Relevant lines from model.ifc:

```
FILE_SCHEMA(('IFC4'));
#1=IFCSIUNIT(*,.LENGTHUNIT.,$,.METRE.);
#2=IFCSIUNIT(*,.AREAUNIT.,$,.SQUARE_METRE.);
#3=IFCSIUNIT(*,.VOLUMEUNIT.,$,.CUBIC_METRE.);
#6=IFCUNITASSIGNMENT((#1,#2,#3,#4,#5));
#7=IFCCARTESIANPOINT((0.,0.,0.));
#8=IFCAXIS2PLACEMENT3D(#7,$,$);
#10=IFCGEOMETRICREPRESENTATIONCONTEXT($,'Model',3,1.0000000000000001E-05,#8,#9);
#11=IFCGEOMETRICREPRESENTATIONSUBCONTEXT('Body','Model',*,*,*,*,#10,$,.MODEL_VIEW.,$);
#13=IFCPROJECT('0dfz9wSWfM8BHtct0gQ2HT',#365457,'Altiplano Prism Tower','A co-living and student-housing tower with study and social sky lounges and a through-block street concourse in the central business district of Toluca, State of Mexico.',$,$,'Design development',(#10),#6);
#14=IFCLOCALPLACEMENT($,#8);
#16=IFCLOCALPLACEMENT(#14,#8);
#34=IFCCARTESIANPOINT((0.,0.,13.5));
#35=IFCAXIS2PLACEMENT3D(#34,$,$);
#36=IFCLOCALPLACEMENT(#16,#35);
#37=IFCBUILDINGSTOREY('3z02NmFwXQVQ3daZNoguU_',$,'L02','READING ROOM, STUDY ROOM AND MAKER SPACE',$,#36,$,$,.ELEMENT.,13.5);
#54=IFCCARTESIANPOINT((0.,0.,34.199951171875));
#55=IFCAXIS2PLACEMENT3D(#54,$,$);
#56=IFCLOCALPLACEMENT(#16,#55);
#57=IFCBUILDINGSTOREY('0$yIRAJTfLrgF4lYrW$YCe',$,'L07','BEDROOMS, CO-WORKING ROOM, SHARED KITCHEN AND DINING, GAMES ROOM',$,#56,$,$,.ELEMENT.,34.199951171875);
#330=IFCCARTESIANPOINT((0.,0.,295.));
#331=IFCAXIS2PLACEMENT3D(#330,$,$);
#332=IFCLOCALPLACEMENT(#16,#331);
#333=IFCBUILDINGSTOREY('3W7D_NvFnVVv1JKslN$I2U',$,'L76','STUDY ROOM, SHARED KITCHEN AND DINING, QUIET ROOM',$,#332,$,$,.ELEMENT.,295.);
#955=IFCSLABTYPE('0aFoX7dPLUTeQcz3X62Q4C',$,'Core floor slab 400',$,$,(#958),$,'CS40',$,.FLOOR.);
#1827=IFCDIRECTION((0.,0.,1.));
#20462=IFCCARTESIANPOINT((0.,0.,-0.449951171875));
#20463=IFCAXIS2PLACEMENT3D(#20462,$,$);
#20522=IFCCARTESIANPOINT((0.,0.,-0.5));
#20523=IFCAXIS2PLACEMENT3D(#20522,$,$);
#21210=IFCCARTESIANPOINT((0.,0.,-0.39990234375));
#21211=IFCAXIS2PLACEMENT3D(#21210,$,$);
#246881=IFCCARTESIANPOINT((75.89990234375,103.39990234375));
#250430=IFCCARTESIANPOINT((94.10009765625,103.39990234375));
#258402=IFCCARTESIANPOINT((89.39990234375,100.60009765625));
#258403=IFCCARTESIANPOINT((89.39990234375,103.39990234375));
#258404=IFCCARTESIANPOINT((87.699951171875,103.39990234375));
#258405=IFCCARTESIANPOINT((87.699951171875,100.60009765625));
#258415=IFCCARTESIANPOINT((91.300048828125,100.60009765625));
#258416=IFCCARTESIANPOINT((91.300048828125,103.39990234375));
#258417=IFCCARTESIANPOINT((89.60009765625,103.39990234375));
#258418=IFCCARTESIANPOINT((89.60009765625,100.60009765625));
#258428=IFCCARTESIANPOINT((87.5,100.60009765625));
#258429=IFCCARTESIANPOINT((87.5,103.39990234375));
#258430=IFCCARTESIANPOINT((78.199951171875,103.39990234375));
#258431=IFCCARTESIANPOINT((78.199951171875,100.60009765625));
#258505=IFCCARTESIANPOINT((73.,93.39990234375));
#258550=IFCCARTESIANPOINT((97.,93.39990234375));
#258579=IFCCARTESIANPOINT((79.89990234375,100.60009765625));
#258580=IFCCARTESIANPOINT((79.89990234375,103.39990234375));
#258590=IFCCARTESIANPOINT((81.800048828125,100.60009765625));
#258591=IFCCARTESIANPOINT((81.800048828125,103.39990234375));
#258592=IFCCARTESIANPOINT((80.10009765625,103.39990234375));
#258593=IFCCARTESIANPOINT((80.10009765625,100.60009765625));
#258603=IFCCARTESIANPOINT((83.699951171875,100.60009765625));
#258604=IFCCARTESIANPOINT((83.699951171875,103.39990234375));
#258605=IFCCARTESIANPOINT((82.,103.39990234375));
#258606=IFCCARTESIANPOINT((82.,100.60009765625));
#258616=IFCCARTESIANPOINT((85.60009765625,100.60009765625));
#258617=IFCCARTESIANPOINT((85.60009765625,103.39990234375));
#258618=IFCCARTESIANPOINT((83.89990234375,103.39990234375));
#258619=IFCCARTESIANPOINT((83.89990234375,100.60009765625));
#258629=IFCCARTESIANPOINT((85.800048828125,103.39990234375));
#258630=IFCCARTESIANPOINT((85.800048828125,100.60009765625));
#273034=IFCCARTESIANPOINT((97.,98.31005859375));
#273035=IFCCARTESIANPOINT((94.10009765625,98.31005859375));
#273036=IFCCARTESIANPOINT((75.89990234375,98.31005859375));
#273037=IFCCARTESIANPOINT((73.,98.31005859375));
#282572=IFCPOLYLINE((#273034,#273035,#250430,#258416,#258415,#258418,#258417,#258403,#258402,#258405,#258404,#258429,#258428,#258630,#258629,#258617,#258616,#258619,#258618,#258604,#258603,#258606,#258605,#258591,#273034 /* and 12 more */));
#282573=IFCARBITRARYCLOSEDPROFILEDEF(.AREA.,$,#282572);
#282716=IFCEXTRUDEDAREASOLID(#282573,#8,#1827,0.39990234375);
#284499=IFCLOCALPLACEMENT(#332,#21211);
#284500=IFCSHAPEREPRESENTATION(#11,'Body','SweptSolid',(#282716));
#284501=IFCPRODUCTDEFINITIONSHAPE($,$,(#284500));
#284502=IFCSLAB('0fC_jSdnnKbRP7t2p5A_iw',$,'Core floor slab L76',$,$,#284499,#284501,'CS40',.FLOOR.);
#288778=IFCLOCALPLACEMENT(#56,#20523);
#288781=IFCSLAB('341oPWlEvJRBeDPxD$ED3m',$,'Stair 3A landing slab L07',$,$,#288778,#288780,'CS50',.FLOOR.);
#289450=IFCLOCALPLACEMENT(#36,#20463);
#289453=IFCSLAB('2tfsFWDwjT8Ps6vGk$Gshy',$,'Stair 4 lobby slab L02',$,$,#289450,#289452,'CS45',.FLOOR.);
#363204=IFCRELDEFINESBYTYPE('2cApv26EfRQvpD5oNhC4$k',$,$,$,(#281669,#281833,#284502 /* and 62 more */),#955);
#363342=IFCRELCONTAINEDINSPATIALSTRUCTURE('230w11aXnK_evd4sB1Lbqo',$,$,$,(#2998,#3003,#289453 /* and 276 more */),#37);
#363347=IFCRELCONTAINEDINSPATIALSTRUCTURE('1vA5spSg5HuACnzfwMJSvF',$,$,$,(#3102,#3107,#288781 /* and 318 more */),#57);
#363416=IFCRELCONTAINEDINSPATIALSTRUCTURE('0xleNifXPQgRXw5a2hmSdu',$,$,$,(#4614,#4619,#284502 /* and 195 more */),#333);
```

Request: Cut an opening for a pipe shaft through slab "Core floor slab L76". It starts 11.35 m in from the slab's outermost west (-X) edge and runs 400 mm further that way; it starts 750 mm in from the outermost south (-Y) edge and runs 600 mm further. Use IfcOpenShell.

```python
import numpy as np
import ifcopenshell
import ifcopenshell.api.feature
import ifcopenshell.api.geometry
import ifcopenshell.api.root
import ifcopenshell.geom
import ifcopenshell.util.placement
import ifcopenshell.util.representation
import ifcopenshell.util.shape
import ifcopenshell.util.unit

model = ifcopenshell.open("model.ifc")
unit_scale = ifcopenshell.util.unit.calculate_unit_scale(model)
settings = ifcopenshell.geom.settings()


def volume(element):
    """Net volume in cubic metres, openings subtracted."""
    shape = ifcopenshell.geom.create_shape(settings, element)
    return ifcopenshell.util.shape.get_volume(shape.geometry)


slab = model.by_guid("0fC_jSdnnKbRP7t2p5A_iw")
before = volume(slab)

# Extent in the slab's own axes, in metres. The edges named are its -X and -Y sides.
slab_shape = ifcopenshell.geom.create_shape(settings, slab)
vertices = ifcopenshell.util.shape.get_vertices(slab_shape.geometry)
x_min, y_min, bottom = vertices.min(axis=0)
top = vertices[:, 2].max()

opening = ifcopenshell.api.root.create_entity(model, ifc_class="IfcOpeningElement", name="Pipe shaft opening", predefined_type="OPENING")
context = ifcopenshell.util.representation.get_context(model, "Model", "Body", "MODEL_VIEW")
width, depth = 0.4, 0.6
outline = [(0.0, 0.0), (width, 0.0), (width, depth), (0.0, depth), (0.0, 0.0)]
# Overshoot both faces by 50 mm so the cut is clean.
shape = ifcopenshell.api.geometry.add_slab_representation(
    model, context=context, depth=top - bottom + 0.1, polyline=outline
)
ifcopenshell.api.geometry.assign_representation(model, product=opening, representation=shape)

matrix = ifcopenshell.util.placement.get_local_placement(slab.ObjectPlacement)
matrix[:, 3] = matrix @ np.append(np.array([x_min + 11.35, y_min + 0.75, bottom - 0.05]) / unit_scale, 1.0)
ifcopenshell.api.geometry.edit_object_placement(model, product=opening, matrix=matrix, is_si=False)
ifcopenshell.api.feature.add_feature(model, feature=opening, element=slab)

after = volume(slab)

print(f"slab volume {before:.3f} -> {after:.3f} m3")

model.write("model_v2.ifc")
```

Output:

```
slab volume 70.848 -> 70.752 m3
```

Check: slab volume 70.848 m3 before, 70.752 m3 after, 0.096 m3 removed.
